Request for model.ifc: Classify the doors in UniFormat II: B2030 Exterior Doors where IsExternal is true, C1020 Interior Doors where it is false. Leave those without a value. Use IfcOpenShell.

First a look at what the model holds.

```python
import ifcopenshell
import ifcopenshell.util.element

model = ifcopenshell.open("model.ifc")
print(model.schema)
print("classifications:", [c.Name for c in model.by_type("IfcClassification")])
values = [ifcopenshell.util.element.get_pset(e, "Pset_DoorCommon", "IsExternal") for e in model.by_type("IfcDoor")]
for value in (True, False, None):
    print("IsExternal", value, values.count(value))
```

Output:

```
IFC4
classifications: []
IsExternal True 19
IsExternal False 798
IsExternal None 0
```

```python
import ifcopenshell
import ifcopenshell.api.classification
import ifcopenshell.util.element

model = ifcopenshell.open("model.ifc")

system = ifcopenshell.api.classification.add_classification(model, classification="UniFormat II")

doors = model.by_type("IfcDoor")
external = {e: ifcopenshell.util.element.get_pset(e, "Pset_DoorCommon", "IsExternal") for e in doors}
for flag, code, name in ((True, "B2030", "Exterior Doors"), (False, "C1020", "Interior Doors")):
    products = [e for e in doors if external[e] is flag]
    ifcopenshell.api.classification.add_reference(
        model, products=products, classification=system, identification=code, name=name
    )
    print(code, len(products))

model.write("model_v2.ifc")
```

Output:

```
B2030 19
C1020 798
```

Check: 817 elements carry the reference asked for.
